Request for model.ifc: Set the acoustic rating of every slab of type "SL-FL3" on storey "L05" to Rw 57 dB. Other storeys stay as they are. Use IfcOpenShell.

First a look at what the model holds.

```python
import ifcopenshell
import ifcopenshell.util.element

model = ifcopenshell.open("model.ifc")
print(model.schema)
storey = next(s for s in model.by_type("IfcBuildingStorey") if s.Name == "L05")
slabs = [e for e in ifcopenshell.util.element.get_decomposition(storey) if e.is_a("IfcSlab")]
seen = {}
for e in slabs:
    element_type = ifcopenshell.util.element.get_type(e)
    key = (element_type.Name if element_type != e and element_type else None, ifcopenshell.util.element.get_pset(e, "Pset_SlabCommon", "AcousticRating"))
    seen[key] = seen.get(key, 0) + 1
for (name, value), count in sorted(seen.items(), key=str):
    print(count, "x", name, "|", value)
```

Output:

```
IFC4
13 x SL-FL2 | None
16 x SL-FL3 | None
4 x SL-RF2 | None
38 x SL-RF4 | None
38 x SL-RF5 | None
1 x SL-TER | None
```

```python
import ifcopenshell
import ifcopenshell.api.pset
import ifcopenshell.util.element

model = ifcopenshell.open("model.ifc")

storey = next(s for s in model.by_type("IfcBuildingStorey") if s.Name == "L05")
slabs = [e for e in ifcopenshell.util.element.get_decomposition(storey) if e.is_a("IfcSlab")]

count = 0
for e in slabs:
    element_type = ifcopenshell.util.element.get_type(e)
    if element_type in (None, e) or element_type.Name != "SL-FL3":
        continue
    # add_pset returns the element's existing set when there is one.
    pset = ifcopenshell.api.pset.add_pset(model, product=e, name="Pset_SlabCommon")
    ifcopenshell.api.pset.edit_pset(model, pset=pset, properties={"AcousticRating": "Rw 57 dB"})
    count += 1

print(count, "slabs updated")

model.write("model_edited.ifc")
```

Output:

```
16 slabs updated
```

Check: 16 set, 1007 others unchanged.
